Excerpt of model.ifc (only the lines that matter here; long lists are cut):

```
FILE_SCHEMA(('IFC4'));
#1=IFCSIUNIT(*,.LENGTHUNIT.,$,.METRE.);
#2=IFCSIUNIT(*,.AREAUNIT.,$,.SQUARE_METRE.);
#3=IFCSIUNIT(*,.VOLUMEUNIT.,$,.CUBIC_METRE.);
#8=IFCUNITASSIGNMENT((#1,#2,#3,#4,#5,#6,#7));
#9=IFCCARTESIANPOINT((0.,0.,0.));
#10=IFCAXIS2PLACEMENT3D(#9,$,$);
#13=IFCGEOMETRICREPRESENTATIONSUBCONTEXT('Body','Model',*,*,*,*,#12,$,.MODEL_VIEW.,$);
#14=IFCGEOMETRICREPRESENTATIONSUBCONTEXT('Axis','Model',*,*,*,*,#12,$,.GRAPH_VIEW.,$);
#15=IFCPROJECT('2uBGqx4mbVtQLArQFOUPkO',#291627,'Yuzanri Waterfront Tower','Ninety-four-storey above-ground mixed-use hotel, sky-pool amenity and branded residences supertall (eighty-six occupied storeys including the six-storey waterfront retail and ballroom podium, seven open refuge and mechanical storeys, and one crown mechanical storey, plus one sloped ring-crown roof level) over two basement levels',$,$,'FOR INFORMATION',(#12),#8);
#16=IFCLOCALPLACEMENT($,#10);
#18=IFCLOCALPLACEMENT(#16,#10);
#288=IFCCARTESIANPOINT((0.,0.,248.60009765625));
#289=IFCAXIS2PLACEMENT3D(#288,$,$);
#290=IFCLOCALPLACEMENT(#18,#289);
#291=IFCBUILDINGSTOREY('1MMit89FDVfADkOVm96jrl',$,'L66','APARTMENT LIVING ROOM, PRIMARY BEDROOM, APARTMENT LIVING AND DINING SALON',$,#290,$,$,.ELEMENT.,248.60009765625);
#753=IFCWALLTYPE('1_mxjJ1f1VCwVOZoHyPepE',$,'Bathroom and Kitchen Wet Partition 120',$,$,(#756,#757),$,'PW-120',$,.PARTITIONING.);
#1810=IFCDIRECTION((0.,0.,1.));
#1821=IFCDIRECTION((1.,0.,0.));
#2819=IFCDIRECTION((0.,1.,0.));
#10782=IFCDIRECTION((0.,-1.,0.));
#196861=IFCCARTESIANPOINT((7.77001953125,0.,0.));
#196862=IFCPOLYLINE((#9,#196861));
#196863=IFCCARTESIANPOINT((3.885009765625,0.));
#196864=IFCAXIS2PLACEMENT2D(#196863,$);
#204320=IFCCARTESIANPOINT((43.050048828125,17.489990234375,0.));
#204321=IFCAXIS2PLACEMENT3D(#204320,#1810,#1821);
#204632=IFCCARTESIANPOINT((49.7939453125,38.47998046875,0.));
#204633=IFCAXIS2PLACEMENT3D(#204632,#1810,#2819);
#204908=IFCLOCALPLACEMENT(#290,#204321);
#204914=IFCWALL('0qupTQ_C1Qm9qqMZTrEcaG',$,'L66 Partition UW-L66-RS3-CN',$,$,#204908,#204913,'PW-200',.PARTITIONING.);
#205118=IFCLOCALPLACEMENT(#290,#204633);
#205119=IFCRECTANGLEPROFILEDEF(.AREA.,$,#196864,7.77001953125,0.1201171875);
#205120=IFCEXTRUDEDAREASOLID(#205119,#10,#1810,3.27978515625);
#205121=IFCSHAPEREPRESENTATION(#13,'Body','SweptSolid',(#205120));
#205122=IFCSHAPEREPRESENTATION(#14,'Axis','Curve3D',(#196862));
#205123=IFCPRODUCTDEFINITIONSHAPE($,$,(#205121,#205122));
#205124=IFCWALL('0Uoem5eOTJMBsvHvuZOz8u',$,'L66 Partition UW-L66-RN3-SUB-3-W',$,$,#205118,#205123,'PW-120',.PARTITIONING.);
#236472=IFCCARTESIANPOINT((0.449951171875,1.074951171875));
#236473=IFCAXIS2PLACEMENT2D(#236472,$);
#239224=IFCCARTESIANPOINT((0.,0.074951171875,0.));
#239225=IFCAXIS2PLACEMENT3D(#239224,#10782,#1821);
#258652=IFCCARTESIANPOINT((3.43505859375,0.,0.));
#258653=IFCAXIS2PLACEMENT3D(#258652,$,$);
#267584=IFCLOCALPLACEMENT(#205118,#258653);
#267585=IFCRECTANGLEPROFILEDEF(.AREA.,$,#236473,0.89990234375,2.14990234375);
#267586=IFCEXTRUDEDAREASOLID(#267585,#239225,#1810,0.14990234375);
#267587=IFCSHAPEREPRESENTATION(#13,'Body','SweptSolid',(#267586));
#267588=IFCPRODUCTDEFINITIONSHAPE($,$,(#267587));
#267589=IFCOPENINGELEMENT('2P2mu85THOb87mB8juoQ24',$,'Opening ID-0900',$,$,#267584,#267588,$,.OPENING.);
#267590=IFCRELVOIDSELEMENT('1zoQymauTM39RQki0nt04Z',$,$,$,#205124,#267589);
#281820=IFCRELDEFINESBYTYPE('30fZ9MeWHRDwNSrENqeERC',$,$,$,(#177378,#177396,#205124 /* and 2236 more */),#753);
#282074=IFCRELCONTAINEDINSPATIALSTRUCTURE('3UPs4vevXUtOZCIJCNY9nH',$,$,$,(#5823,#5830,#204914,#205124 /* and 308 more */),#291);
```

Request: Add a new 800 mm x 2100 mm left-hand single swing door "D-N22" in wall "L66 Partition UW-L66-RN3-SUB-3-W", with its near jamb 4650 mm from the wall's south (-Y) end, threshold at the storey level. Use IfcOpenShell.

```python
import numpy as np
import ifcopenshell
import ifcopenshell.api.feature
import ifcopenshell.api.geometry
import ifcopenshell.api.root
import ifcopenshell.api.spatial
import ifcopenshell.geom
import ifcopenshell.util.element
import ifcopenshell.util.placement
import ifcopenshell.util.representation
import ifcopenshell.util.shape
import ifcopenshell.util.unit

model = ifcopenshell.open("model.ifc")
unit_scale = ifcopenshell.util.unit.calculate_unit_scale(model)
settings = ifcopenshell.geom.settings()


def volume(element):
    """Net volume in cubic metres, openings subtracted."""
    shape = ifcopenshell.geom.create_shape(settings, element)
    return ifcopenshell.util.shape.get_volume(shape.geometry)


wall = model.by_id(205124)
storey = ifcopenshell.util.element.get_container(wall, ifc_class="IfcBuildingStorey")
context = ifcopenshell.util.representation.get_context(model, "Model", "Body", "MODEL_VIEW")
before = volume(wall)

width, height, from_end, sill = 0.8, 2.1, 4.65, 0.0  # metres

# The wall runs along its own X axis, and the end named is its -X end.
wall_shape = ifcopenshell.geom.create_shape(settings, wall)
x, y, z = ifcopenshell.util.shape.get_vertices(wall_shape.geometry).T
start = x.min() + from_end
face, thickness = float(y.min()), float(y.max() - y.min())
wall_matrix = ifcopenshell.util.placement.get_local_placement(wall.ObjectPlacement)
level = ifcopenshell.util.placement.get_local_placement(storey.ObjectPlacement)[2, 3]


def in_wall(x, y):
    """Placement at x, y metres in the wall's axes, at sill height."""
    matrix = wall_matrix.copy()
    matrix[:, 3] = wall_matrix @ np.array([x / unit_scale, y / unit_scale, 0.0, 1.0])
    matrix[2, 3] = level + sill / unit_scale
    return matrix


# Opening: a box that overshoots both wall faces by 50 mm.
opening = ifcopenshell.api.root.create_entity(model, ifc_class="IfcOpeningElement", predefined_type="OPENING")
box = ifcopenshell.api.geometry.add_wall_representation(
    model, context=context, length=width, height=height, thickness=thickness + 0.1
)
ifcopenshell.api.geometry.assign_representation(model, product=opening, representation=box)
ifcopenshell.api.geometry.edit_object_placement(model, product=opening, matrix=in_wall(start, face - 0.05), is_si=False)
ifcopenshell.api.feature.add_feature(model, feature=opening, element=wall)

door = ifcopenshell.api.root.create_entity(model, ifc_class="IfcDoor", name="D-N22", predefined_type="DOOR")
door.OverallWidth, door.OverallHeight = width / unit_scale, height / unit_scale
door.OperationType = "SINGLE_SWING_LEFT"
body = ifcopenshell.api.geometry.add_door_representation(
    model,
    context=context,
    overall_width=door.OverallWidth,
    overall_height=door.OverallHeight,
    operation_type="SINGLE_SWING_LEFT",
    lining_properties={"LiningDepth": thickness / unit_scale, "ThresholdDepth": thickness / unit_scale},
)
ifcopenshell.api.geometry.assign_representation(model, product=door, representation=body)
ifcopenshell.api.spatial.assign_container(model, products=[door], relating_structure=storey)
ifcopenshell.api.feature.add_filling(model, opening=opening, element=door)

# The lining spans the wall, so the door starts at the wall face.
ifcopenshell.api.geometry.edit_object_placement(model, product=door, matrix=in_wall(start, face), is_si=False)

after = volume(wall)

print(f"wall volume {before:.3f} -> {after:.3f} m3")

model.write("model_edited.ifc")
```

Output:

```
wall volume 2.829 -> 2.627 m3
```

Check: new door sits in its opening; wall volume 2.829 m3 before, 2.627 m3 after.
